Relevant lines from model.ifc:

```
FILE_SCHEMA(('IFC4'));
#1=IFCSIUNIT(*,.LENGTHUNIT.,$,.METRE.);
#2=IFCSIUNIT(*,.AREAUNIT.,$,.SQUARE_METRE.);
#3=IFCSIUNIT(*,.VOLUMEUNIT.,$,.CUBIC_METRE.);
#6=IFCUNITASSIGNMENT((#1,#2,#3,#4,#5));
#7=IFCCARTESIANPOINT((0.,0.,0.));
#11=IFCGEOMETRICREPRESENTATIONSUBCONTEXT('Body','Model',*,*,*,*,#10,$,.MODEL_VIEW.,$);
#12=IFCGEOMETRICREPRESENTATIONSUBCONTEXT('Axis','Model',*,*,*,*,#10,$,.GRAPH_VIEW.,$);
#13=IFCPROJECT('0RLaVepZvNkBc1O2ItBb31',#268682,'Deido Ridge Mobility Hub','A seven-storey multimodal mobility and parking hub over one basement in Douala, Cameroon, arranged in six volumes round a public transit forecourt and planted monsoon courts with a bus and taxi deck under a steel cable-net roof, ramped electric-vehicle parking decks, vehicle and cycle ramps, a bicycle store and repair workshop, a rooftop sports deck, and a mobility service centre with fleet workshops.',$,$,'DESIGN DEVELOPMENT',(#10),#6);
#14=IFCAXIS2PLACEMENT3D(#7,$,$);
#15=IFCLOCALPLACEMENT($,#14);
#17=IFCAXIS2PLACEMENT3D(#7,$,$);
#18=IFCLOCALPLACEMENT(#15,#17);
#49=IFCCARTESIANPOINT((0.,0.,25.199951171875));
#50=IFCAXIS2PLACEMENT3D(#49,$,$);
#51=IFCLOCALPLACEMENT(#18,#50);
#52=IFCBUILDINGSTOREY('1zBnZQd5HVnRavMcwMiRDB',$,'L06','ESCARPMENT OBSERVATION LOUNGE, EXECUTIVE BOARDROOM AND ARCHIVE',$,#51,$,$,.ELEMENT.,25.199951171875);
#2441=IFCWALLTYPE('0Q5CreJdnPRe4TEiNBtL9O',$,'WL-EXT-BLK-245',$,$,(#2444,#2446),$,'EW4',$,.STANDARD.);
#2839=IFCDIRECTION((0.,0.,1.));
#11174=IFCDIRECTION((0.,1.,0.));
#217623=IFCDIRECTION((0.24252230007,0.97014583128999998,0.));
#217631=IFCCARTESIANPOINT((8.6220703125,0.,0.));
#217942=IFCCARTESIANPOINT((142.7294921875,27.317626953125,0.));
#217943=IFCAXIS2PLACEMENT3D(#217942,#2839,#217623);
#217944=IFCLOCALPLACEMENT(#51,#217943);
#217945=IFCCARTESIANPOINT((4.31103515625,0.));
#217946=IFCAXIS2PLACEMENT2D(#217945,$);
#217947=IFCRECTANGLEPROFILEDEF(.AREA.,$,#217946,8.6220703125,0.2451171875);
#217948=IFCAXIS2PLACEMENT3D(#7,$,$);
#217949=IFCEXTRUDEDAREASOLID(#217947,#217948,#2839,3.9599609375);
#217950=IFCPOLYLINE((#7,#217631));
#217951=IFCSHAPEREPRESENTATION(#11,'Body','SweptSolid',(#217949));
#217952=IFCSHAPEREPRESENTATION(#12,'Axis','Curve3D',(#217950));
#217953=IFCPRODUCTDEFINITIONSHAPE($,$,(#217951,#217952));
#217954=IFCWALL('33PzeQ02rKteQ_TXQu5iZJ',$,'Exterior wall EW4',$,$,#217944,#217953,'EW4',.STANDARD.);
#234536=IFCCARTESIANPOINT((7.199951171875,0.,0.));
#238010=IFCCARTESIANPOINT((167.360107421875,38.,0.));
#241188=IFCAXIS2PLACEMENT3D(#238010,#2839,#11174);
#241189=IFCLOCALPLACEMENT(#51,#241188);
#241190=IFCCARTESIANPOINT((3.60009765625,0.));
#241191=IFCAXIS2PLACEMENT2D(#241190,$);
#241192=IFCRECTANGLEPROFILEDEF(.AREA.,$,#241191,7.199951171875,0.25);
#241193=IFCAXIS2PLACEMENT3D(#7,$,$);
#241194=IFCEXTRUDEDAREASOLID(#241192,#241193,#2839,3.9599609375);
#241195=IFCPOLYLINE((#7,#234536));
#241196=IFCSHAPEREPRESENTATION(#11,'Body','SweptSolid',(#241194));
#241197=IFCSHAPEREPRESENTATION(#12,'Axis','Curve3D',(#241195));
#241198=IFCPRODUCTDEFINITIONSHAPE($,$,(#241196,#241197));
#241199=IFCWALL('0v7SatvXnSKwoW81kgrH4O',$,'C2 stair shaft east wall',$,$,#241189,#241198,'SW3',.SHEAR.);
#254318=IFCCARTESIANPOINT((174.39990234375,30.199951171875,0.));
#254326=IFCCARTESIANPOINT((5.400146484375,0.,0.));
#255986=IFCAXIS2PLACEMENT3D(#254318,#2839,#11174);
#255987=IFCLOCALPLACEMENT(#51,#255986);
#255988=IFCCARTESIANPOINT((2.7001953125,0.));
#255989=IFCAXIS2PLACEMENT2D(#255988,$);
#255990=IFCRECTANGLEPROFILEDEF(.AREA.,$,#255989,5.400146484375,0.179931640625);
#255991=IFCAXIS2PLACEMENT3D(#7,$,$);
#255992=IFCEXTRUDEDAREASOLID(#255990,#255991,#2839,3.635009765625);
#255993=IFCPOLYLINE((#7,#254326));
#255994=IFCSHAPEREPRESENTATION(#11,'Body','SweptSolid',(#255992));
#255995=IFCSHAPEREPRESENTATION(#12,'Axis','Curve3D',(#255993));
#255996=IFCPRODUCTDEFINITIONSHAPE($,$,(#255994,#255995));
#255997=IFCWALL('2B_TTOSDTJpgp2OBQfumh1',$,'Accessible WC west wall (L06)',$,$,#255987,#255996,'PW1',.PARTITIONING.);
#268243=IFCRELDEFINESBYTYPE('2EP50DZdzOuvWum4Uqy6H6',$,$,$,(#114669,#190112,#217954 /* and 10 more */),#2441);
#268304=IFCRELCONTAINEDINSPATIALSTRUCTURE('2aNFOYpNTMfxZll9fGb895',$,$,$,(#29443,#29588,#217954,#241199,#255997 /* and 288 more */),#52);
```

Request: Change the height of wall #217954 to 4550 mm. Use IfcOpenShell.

```python
import ifcopenshell
import ifcopenshell.geom
import ifcopenshell.util.representation
import ifcopenshell.util.shape

model = ifcopenshell.open("model.ifc")
settings = ifcopenshell.geom.settings()


def volume(element):
    """Net volume in cubic metres, openings subtracted."""
    shape = ifcopenshell.geom.create_shape(settings, element)
    return ifcopenshell.util.shape.get_volume(shape.geometry)


wall = model.by_guid("33PzeQ02rKteQ_TXQu5iZJ")
before = volume(wall)

body = ifcopenshell.util.representation.get_representation(wall, "Model", "Body")
solid = body.Items[0]
old_height = solid.Depth
solid.Depth = 4.55
after = volume(wall)

print(f"height {old_height:g} -> {solid.Depth:g}, volume {before:.3f} -> {after:.3f} m3")

model.write("model_edited.ifc")
```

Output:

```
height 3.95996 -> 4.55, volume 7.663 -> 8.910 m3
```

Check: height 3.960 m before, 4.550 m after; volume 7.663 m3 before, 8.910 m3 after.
